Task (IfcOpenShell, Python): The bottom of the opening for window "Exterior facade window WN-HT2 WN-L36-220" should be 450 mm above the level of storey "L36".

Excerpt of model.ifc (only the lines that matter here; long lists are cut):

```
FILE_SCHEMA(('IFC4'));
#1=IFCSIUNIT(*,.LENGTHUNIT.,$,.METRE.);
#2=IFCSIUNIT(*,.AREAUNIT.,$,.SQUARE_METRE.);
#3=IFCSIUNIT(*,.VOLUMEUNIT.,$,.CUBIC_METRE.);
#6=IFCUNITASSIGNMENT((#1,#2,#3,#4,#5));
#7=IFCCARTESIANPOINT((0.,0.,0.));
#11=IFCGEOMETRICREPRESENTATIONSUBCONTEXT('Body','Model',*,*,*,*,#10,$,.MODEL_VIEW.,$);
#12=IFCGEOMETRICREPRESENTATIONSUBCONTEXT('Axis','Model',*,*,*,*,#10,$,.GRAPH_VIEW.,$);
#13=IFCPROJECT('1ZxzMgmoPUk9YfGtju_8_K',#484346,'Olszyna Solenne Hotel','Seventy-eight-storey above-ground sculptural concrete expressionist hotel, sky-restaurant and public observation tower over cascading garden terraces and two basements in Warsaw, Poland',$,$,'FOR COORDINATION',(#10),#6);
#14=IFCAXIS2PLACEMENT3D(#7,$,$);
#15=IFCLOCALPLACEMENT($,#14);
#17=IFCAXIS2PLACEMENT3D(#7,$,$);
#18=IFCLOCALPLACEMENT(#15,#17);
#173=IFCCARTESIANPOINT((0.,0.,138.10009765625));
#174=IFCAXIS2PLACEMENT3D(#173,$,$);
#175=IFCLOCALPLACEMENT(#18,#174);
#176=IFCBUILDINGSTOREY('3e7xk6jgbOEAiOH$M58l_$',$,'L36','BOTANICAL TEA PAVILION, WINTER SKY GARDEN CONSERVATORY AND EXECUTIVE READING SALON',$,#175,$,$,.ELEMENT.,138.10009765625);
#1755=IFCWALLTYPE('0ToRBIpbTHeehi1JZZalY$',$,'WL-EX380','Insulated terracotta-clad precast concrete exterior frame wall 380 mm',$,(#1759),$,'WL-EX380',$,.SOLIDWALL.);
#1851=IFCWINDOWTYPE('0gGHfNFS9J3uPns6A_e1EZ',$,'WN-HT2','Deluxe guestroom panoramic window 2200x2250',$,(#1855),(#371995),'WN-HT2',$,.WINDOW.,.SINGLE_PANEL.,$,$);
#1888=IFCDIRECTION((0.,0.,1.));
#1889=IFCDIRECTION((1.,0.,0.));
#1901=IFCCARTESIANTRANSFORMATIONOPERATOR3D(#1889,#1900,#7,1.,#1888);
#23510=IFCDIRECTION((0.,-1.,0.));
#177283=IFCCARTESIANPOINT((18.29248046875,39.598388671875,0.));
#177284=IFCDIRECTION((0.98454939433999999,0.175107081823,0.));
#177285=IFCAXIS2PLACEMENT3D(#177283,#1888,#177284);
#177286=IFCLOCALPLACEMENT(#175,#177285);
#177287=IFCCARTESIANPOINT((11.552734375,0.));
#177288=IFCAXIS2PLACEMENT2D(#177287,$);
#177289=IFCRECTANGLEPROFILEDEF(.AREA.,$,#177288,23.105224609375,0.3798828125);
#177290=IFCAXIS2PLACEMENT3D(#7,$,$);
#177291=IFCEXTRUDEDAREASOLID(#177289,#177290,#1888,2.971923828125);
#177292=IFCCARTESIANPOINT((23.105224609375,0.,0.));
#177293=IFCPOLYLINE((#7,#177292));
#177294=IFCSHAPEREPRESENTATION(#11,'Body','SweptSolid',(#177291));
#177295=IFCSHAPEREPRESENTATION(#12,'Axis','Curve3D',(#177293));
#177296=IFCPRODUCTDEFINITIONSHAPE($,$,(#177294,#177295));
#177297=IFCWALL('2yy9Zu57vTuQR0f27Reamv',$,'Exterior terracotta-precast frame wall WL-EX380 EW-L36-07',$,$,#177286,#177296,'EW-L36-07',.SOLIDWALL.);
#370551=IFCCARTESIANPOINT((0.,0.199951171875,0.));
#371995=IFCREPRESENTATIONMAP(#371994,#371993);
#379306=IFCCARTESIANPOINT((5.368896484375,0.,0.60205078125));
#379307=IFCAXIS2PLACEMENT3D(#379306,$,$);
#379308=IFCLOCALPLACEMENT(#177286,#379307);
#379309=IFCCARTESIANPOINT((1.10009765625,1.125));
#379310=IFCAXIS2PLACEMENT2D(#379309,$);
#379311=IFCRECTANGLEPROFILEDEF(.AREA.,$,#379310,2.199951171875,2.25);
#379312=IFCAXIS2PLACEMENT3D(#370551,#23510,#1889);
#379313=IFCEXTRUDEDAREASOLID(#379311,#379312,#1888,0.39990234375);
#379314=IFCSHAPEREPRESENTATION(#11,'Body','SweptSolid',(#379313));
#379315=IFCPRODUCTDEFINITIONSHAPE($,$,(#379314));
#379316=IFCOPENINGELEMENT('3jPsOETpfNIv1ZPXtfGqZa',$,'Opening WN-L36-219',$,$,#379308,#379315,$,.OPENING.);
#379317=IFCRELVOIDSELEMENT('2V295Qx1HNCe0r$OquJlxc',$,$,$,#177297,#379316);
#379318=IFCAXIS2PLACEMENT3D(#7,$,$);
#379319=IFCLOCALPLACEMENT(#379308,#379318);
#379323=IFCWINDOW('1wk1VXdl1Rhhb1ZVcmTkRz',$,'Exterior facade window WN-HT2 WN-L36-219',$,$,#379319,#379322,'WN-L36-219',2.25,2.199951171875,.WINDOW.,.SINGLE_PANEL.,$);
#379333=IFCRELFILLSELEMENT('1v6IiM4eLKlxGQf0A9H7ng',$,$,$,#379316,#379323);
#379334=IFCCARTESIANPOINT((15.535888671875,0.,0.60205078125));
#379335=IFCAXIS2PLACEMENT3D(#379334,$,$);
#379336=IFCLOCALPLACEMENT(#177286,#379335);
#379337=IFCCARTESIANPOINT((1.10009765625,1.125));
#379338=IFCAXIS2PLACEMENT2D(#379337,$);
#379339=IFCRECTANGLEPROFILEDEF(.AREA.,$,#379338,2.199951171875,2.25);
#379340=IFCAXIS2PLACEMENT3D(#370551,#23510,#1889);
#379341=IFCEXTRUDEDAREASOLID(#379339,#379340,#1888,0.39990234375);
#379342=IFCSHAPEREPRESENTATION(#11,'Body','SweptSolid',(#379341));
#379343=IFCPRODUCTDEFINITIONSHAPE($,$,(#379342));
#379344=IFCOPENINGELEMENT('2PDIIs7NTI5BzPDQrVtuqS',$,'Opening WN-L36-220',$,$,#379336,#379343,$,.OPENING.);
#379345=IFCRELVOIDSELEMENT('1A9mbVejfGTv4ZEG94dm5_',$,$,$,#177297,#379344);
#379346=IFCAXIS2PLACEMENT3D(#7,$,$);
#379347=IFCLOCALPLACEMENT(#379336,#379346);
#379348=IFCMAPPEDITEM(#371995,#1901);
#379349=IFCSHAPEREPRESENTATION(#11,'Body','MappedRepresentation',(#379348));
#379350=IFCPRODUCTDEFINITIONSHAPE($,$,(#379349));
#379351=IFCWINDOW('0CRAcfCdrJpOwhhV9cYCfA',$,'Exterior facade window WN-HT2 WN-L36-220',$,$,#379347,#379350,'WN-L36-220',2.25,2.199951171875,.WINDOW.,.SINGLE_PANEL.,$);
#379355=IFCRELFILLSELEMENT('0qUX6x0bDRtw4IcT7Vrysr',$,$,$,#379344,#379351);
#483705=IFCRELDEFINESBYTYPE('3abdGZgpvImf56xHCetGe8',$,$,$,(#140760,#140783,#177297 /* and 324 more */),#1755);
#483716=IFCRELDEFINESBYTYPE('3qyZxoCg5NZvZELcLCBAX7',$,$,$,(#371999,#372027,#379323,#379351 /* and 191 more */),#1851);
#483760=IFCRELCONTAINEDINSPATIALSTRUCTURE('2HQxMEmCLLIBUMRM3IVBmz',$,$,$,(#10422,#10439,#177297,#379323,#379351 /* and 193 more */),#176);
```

```python
import numpy as np
import ifcopenshell
import ifcopenshell.api.geometry
import ifcopenshell.geom
import ifcopenshell.util.element
import ifcopenshell.util.placement
import ifcopenshell.util.shape
import ifcopenshell.util.unit

model = ifcopenshell.open("model.ifc")
unit_scale = ifcopenshell.util.unit.calculate_unit_scale(model)

window = model.by_guid("0CRAcfCdrJpOwhhV9cYCfA")
opening = window.FillsVoids[0].RelatingOpeningElement
storey = ifcopenshell.util.element.get_container(window, ifc_class="IfcBuildingStorey")
level = ifcopenshell.util.placement.get_local_placement(storey.ObjectPlacement)[2, 3]

# The opening's origin need not be at the sill, so measure its lowest point.
shape = ifcopenshell.geom.create_shape(ifcopenshell.geom.settings(), opening)
bottom = ifcopenshell.util.shape.get_shape_bottom_elevation(shape, shape.geometry) / unit_scale
dz = level + 0.45 / unit_scale - bottom

shift = np.array([0.0, 0.0, dz])
# The window is placed relative to its opening, so it follows when the opening moves.
matrix = ifcopenshell.util.placement.get_local_placement(opening.ObjectPlacement)
matrix[:3, 3] += shift
ifcopenshell.api.geometry.edit_object_placement(
    model, product=opening, matrix=matrix, is_si=False, should_transform_children=True
)

print(f"moved by {dz * unit_scale:+.3f} m")

model.write("model_v2.ifc")
```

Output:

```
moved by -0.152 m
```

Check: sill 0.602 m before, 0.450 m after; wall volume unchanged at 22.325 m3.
